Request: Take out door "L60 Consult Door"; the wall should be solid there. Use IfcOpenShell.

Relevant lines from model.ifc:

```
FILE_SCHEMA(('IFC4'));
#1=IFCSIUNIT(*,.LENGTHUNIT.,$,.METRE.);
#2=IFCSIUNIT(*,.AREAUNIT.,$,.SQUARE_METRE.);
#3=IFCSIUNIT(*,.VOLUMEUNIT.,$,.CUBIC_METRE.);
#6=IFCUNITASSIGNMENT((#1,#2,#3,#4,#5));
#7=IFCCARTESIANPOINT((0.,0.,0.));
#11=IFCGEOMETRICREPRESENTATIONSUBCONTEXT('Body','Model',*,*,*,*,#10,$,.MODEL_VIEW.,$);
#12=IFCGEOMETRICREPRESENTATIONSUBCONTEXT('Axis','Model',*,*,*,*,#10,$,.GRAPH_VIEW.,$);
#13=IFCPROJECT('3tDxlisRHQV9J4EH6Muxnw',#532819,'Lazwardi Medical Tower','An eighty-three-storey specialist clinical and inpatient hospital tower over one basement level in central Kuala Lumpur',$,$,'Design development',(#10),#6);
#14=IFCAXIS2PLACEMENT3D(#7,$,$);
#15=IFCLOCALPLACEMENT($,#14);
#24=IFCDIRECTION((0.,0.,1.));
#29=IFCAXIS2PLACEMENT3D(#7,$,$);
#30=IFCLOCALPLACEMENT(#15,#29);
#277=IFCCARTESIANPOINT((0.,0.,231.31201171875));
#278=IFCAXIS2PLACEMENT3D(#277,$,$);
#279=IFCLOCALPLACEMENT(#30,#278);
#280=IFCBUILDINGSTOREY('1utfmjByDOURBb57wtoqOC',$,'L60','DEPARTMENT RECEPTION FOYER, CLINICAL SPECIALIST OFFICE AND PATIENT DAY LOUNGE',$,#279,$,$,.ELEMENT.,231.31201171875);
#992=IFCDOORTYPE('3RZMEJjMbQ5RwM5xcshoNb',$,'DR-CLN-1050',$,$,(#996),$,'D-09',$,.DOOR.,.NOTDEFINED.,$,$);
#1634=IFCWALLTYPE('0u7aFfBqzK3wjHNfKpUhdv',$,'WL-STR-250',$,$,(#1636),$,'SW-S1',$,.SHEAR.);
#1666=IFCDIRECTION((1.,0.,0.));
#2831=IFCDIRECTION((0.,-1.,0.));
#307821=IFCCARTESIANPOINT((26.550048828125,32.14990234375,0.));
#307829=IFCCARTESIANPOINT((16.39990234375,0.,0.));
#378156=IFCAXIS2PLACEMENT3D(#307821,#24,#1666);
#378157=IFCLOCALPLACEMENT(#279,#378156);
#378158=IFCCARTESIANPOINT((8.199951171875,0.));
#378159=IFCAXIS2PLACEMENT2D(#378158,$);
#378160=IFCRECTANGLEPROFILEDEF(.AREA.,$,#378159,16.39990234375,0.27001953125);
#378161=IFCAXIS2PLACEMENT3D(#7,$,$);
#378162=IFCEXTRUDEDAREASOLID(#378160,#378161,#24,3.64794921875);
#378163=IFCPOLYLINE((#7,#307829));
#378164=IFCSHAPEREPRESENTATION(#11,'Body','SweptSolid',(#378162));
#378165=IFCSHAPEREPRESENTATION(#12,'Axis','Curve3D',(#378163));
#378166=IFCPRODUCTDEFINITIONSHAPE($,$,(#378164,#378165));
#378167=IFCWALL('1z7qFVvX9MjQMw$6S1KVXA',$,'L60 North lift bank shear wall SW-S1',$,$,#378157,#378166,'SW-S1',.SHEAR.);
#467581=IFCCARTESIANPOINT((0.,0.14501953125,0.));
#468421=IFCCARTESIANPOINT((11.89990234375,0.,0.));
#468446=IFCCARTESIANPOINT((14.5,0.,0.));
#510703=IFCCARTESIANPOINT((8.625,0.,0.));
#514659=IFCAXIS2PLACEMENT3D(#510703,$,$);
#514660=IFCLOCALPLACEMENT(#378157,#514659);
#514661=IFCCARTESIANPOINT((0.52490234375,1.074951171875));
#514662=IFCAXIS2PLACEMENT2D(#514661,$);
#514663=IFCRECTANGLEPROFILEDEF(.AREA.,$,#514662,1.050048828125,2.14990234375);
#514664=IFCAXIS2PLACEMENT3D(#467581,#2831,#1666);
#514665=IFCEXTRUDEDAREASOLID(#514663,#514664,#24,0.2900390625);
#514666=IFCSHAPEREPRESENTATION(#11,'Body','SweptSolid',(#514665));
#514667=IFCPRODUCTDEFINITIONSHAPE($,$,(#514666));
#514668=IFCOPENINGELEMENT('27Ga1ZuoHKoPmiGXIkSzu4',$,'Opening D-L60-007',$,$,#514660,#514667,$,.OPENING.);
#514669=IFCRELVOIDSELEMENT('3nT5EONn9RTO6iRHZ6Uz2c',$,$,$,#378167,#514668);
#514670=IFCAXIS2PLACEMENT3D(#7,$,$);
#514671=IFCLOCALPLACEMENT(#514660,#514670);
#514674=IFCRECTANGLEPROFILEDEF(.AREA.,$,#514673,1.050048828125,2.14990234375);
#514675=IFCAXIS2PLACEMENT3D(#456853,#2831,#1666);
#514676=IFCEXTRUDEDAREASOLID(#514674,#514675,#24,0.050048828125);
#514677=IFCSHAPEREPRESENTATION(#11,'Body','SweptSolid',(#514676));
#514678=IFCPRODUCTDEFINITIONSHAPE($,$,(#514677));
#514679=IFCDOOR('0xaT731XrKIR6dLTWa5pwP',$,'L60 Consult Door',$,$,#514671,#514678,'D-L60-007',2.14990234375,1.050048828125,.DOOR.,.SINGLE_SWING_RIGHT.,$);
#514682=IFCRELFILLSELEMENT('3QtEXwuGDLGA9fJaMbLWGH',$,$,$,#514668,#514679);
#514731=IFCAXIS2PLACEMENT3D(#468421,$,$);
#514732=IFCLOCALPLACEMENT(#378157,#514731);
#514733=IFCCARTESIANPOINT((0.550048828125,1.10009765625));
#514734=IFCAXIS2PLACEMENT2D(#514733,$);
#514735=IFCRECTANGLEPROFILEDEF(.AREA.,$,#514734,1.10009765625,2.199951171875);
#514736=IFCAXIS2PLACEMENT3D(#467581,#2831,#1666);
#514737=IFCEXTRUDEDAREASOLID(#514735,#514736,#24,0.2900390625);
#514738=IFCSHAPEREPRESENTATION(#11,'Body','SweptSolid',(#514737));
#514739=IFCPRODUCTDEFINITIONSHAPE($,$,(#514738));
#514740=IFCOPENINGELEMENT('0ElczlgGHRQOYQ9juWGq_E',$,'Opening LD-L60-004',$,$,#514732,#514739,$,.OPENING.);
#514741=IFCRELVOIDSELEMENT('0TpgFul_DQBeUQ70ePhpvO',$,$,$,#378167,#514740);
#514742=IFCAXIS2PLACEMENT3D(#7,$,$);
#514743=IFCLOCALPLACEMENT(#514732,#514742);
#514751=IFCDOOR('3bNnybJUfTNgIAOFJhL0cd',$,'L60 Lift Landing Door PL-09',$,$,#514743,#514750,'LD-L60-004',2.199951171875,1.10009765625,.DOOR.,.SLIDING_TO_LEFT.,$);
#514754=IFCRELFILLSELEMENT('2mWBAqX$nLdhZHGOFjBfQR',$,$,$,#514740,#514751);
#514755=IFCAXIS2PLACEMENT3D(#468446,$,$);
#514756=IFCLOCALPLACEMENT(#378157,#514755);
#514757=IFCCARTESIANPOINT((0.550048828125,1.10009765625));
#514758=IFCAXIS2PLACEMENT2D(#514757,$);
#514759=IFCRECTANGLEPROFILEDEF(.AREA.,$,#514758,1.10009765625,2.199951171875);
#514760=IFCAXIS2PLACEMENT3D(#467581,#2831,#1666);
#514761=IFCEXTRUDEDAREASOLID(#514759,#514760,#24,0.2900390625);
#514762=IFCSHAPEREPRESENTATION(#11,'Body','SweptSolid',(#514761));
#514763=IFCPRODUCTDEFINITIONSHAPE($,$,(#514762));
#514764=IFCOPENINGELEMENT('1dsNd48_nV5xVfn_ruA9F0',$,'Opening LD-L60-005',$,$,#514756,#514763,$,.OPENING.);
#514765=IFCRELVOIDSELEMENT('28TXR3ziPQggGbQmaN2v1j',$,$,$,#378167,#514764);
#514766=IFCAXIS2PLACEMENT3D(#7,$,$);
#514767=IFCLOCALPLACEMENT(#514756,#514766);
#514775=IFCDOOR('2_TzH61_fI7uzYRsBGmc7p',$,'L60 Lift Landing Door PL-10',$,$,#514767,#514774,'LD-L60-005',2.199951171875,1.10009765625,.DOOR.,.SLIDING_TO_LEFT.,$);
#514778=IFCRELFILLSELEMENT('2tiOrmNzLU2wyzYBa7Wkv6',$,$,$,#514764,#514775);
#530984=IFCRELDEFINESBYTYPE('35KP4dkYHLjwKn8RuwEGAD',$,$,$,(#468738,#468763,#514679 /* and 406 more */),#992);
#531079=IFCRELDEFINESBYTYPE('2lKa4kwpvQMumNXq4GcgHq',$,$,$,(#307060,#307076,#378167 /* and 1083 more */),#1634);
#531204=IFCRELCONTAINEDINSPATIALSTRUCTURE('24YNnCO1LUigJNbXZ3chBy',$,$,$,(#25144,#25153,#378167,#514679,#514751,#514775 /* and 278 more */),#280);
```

```python
import ifcopenshell
import ifcopenshell.api.feature
import ifcopenshell.api.root
import ifcopenshell.geom
import ifcopenshell.util.shape

model = ifcopenshell.open("model.ifc")
settings = ifcopenshell.geom.settings()


def volume(element):
    """Net volume in cubic metres, openings subtracted."""
    shape = ifcopenshell.geom.create_shape(settings, element)
    return ifcopenshell.util.shape.get_volume(shape.geometry)


door = model.by_guid("0xaT731XrKIR6dLTWa5pwP")
opening = door.FillsVoids[0].RelatingOpeningElement
wall = opening.VoidsElements[0].RelatingBuildingElement
before = volume(wall)

ifcopenshell.api.root.remove_product(model, product=door)
ifcopenshell.api.feature.remove_feature(model, feature=opening)

after = volume(wall)

print(f"wall volume {before:.3f} -> {after:.3f} m3")

model.write("model_v2.ifc")
```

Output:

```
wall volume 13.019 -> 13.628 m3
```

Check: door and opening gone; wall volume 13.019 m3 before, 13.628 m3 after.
